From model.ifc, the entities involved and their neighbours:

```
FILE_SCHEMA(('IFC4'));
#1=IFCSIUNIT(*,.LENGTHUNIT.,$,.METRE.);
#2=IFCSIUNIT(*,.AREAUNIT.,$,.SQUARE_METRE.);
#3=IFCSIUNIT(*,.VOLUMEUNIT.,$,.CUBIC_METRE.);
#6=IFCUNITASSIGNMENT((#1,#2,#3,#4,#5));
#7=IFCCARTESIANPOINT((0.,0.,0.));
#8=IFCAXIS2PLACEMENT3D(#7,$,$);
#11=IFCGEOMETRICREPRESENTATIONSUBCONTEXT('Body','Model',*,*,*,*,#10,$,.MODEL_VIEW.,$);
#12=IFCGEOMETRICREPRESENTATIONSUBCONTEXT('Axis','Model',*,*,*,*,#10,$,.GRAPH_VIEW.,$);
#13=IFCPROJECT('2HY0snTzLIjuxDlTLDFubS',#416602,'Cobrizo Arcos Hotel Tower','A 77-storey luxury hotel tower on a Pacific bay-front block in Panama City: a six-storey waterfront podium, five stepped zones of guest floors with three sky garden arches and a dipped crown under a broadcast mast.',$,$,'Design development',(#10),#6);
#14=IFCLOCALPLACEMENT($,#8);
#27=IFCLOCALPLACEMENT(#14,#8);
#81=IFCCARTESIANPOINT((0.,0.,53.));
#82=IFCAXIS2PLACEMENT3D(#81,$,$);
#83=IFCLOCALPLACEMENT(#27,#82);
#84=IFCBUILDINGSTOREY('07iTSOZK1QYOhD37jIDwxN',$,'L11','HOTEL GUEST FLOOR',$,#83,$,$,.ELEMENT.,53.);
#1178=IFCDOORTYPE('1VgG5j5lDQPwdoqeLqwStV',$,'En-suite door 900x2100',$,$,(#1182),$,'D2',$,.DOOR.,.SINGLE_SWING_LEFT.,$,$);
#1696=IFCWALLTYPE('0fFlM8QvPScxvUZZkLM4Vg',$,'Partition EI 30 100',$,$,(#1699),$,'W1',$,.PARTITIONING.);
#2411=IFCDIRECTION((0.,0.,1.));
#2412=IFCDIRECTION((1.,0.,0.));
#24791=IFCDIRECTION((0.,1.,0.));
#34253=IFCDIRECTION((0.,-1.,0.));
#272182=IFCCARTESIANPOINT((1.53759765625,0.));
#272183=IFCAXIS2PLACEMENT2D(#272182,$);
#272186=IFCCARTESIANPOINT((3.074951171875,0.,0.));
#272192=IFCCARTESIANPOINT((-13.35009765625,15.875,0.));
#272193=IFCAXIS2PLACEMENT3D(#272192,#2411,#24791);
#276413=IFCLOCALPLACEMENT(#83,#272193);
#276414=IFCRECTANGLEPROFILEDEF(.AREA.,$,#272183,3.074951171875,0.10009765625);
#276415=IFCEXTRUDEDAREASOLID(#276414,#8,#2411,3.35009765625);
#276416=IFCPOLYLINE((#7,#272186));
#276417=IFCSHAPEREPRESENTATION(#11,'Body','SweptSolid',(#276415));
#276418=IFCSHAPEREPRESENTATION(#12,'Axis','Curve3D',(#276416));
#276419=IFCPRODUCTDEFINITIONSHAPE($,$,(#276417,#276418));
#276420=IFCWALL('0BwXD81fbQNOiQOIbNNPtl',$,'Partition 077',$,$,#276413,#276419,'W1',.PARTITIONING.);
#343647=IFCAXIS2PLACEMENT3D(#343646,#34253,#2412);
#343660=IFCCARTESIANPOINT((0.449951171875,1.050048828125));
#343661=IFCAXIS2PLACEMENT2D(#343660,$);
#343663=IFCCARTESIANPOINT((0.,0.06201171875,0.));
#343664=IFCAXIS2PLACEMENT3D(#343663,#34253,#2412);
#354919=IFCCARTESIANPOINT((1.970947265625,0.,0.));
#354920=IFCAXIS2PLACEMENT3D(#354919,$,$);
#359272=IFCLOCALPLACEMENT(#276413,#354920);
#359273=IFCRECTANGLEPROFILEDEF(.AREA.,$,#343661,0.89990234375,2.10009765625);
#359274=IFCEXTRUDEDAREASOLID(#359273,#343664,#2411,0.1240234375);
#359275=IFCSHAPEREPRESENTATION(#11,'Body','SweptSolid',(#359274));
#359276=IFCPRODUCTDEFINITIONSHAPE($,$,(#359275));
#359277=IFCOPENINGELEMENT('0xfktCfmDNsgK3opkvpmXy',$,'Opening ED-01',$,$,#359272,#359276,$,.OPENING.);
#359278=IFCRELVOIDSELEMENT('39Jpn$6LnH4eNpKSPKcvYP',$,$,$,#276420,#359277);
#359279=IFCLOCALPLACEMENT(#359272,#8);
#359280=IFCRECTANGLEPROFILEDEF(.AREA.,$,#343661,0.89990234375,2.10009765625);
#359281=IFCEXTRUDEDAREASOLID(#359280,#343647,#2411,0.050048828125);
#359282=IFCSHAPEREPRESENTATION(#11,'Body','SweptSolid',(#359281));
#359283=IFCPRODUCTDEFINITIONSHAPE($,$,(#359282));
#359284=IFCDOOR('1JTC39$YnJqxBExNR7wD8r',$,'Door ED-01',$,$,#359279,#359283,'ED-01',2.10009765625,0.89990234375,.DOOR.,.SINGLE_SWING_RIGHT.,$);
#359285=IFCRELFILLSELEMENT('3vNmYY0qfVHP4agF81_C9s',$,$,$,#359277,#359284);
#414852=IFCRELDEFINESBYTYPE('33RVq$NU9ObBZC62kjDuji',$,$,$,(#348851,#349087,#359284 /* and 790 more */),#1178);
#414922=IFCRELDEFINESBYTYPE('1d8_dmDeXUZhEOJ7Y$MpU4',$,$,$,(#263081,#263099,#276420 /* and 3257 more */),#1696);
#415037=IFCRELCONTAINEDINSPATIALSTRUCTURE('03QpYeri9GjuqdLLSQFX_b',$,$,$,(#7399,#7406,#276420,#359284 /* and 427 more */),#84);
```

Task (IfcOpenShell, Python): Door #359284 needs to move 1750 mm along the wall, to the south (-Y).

```python
import ifcopenshell
import ifcopenshell.api.geometry
import ifcopenshell.util.placement
import ifcopenshell.util.unit

model = ifcopenshell.open("model.ifc")
unit_scale = ifcopenshell.util.unit.calculate_unit_scale(model)

door = model.by_id(359284)
opening = door.FillsVoids[0].RelatingOpeningElement
wall = opening.VoidsElements[0].RelatingBuildingElement

wall_matrix = ifcopenshell.util.placement.get_local_placement(wall.ObjectPlacement)
shift = wall_matrix[:3, 0] * -1.75 / unit_scale
before = ifcopenshell.util.placement.get_local_placement(door.ObjectPlacement)[:3, 3].copy()

# The door is placed relative to its opening, so it follows when the opening moves.
matrix = ifcopenshell.util.placement.get_local_placement(opening.ObjectPlacement)
matrix[:3, 3] += shift
ifcopenshell.api.geometry.edit_object_placement(
    model, product=opening, matrix=matrix, is_si=False, should_transform_children=True
)

after = ifcopenshell.util.placement.get_local_placement(door.ObjectPlacement)[:3, 3]
print("door moved by", (after - before).round(3) + 0.0)

model.write("model-out.ifc")
```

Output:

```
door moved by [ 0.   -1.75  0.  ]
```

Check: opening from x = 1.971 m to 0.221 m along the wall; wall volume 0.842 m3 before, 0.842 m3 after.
